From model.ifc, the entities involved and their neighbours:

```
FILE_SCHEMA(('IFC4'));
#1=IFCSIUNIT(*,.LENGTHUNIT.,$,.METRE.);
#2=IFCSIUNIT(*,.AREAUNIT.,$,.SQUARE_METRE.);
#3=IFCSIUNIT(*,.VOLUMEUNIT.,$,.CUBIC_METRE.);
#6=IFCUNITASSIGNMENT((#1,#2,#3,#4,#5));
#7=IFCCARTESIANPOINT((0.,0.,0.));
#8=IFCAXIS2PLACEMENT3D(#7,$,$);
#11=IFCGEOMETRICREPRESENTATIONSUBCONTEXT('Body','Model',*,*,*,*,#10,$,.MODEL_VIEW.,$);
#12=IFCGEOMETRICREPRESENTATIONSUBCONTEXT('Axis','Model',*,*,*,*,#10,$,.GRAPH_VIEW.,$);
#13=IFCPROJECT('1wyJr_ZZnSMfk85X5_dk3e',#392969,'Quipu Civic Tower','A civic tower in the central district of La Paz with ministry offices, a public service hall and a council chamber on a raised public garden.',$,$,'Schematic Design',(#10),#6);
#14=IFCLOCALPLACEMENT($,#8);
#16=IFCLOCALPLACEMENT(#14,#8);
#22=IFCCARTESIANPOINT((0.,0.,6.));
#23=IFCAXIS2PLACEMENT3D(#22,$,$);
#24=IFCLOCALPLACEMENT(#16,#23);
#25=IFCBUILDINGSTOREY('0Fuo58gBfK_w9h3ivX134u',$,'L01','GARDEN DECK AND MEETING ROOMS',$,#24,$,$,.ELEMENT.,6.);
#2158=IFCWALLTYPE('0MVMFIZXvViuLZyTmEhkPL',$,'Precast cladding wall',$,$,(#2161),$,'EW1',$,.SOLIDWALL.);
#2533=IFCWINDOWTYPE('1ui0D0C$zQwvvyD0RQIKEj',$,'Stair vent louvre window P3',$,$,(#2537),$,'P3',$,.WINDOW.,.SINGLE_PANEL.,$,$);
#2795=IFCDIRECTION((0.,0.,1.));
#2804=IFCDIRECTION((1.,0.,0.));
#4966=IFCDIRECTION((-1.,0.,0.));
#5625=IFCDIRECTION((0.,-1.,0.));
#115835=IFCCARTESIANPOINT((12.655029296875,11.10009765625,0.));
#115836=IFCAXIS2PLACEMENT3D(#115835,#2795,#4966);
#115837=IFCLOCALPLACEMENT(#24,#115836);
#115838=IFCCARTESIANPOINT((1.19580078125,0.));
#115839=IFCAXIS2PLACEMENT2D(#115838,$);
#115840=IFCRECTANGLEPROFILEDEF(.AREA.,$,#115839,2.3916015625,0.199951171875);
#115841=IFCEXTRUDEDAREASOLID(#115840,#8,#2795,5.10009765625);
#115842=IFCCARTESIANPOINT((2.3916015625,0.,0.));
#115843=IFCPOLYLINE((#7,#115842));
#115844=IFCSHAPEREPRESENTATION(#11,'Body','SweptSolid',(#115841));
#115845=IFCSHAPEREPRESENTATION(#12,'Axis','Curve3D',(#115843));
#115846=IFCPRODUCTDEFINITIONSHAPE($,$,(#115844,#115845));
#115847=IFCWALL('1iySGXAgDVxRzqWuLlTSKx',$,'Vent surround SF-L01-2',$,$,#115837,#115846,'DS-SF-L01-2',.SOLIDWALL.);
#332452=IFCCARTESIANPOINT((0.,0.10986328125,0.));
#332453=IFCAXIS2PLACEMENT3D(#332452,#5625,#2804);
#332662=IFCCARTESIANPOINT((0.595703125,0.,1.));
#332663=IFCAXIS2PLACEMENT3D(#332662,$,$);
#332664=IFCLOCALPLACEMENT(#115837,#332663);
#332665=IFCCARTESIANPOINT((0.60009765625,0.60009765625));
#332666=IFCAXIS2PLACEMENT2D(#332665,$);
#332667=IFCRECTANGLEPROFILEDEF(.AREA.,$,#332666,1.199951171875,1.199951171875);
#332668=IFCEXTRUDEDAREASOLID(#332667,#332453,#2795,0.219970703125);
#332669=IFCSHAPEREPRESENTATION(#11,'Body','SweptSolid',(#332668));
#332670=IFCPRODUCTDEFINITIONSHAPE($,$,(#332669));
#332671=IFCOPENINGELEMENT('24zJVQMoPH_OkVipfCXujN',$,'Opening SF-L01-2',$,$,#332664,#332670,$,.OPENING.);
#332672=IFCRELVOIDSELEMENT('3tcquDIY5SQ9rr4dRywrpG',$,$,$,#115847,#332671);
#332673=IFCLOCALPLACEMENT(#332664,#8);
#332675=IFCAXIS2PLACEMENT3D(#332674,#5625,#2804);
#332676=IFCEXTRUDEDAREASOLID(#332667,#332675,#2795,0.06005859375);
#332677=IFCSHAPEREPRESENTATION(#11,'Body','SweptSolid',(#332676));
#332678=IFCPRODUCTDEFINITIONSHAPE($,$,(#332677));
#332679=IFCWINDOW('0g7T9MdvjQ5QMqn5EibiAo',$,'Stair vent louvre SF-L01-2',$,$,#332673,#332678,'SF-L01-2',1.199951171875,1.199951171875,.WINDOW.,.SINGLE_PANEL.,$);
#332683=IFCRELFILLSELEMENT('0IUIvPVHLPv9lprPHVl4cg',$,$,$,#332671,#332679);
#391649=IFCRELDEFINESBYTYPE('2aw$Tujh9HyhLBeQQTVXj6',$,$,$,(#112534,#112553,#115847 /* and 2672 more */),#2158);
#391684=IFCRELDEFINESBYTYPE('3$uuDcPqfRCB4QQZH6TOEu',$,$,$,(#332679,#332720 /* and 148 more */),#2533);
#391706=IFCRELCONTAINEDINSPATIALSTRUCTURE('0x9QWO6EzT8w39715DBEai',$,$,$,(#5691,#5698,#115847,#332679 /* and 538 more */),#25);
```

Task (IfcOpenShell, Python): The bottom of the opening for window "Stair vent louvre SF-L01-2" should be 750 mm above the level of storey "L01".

```python
import numpy as np
import ifcopenshell
import ifcopenshell.api.geometry
import ifcopenshell.geom
import ifcopenshell.util.element
import ifcopenshell.util.placement
import ifcopenshell.util.shape
import ifcopenshell.util.unit

model = ifcopenshell.open("model.ifc")
unit_scale = ifcopenshell.util.unit.calculate_unit_scale(model)

window = model.by_guid("0g7T9MdvjQ5QMqn5EibiAo")
opening = window.FillsVoids[0].RelatingOpeningElement
storey = ifcopenshell.util.element.get_container(window, ifc_class="IfcBuildingStorey")
level = ifcopenshell.util.placement.get_local_placement(storey.ObjectPlacement)[2, 3]

# The opening's origin need not be at the sill, so measure its lowest point.
shape = ifcopenshell.geom.create_shape(ifcopenshell.geom.settings(), opening)
bottom = ifcopenshell.util.shape.get_shape_bottom_elevation(shape, shape.geometry) / unit_scale
dz = level + 0.75 / unit_scale - bottom

shift = np.array([0.0, 0.0, dz])
# The window is placed relative to its opening, so it follows when the opening moves.
matrix = ifcopenshell.util.placement.get_local_placement(opening.ObjectPlacement)
matrix[:3, 3] += shift
ifcopenshell.api.geometry.edit_object_placement(
    model, product=opening, matrix=matrix, is_si=False, should_transform_children=True
)

print(f"moved by {dz * unit_scale:+.3f} m")

model.write("model_updated.ifc")
```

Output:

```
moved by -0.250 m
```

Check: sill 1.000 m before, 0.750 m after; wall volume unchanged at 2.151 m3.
